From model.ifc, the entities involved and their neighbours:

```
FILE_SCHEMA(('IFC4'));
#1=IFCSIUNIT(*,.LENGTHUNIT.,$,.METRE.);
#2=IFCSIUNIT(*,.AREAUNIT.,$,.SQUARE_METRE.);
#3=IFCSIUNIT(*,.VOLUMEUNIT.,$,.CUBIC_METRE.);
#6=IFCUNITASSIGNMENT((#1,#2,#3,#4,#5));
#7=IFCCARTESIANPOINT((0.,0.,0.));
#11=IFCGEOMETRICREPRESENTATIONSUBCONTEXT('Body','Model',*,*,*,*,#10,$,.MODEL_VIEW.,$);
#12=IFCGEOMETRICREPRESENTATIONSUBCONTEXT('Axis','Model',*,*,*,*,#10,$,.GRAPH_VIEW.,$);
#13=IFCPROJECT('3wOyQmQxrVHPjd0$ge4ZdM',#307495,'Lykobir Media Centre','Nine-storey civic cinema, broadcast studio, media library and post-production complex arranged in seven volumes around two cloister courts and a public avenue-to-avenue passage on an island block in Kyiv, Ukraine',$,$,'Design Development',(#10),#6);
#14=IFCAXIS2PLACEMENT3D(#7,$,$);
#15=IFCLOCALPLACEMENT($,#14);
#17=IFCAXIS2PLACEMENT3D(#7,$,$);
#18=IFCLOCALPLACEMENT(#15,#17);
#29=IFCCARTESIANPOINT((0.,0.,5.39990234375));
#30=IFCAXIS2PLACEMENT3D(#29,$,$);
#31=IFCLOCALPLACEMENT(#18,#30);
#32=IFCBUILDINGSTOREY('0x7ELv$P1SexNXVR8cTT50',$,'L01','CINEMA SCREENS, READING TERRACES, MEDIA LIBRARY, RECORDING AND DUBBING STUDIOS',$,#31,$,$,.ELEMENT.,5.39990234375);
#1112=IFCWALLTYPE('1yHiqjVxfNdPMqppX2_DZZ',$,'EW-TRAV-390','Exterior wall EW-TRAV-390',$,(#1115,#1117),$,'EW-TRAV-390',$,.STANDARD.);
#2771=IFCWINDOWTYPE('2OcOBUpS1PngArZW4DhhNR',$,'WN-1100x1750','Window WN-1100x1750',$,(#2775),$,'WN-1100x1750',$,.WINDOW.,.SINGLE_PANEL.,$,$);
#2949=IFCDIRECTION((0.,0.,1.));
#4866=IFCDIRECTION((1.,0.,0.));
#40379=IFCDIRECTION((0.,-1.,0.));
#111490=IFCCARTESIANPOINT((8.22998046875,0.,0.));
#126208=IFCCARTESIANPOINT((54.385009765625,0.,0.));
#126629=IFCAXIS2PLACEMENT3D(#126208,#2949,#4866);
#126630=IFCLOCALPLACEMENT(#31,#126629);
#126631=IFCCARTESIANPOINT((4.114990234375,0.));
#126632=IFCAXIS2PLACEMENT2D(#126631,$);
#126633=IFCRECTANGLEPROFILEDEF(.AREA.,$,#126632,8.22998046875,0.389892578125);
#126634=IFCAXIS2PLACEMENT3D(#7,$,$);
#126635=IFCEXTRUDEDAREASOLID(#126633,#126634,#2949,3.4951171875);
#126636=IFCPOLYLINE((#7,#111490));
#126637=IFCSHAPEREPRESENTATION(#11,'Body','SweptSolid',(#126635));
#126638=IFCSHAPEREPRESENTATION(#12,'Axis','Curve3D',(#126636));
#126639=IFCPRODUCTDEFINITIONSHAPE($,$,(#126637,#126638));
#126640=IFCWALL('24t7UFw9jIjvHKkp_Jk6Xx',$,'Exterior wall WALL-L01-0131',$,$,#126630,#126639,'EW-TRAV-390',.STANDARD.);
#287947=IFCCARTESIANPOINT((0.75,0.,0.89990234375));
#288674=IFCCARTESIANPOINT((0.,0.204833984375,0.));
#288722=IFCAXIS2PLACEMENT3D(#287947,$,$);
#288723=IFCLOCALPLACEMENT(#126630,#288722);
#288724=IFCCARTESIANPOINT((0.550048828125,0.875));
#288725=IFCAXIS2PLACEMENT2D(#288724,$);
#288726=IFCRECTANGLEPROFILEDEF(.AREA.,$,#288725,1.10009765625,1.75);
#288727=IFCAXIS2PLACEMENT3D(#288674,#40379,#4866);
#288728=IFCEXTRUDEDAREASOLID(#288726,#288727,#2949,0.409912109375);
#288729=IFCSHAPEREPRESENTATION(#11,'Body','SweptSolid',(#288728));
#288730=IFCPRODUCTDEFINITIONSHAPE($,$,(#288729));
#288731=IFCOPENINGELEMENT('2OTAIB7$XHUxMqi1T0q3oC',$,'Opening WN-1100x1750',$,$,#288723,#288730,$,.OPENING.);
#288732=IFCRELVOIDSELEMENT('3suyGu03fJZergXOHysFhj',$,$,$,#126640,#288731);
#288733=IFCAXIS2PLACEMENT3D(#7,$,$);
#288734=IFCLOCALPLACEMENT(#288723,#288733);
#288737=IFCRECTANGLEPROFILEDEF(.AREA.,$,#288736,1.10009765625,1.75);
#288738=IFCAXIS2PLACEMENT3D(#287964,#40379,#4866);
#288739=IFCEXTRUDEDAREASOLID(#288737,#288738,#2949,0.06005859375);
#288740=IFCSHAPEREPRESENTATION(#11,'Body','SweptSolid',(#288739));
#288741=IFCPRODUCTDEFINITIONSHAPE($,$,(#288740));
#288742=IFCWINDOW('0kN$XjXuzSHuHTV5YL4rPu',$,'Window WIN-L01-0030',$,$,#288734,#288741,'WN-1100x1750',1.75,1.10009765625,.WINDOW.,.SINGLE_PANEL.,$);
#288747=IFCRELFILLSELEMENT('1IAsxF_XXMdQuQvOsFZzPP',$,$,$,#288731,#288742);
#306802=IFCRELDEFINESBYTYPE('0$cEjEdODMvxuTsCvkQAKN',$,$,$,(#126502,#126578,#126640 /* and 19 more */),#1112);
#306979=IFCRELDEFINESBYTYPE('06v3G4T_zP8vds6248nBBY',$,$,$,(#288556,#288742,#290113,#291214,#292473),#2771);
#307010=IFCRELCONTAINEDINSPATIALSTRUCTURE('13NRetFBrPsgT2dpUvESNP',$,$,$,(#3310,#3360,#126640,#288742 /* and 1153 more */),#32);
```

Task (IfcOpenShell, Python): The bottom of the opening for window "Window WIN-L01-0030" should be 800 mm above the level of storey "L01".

```python
import numpy as np
import ifcopenshell
import ifcopenshell.api.geometry
import ifcopenshell.geom
import ifcopenshell.util.element
import ifcopenshell.util.placement
import ifcopenshell.util.shape
import ifcopenshell.util.unit

model = ifcopenshell.open("model.ifc")
unit_scale = ifcopenshell.util.unit.calculate_unit_scale(model)

window = model.by_guid("0kN$XjXuzSHuHTV5YL4rPu")
opening = window.FillsVoids[0].RelatingOpeningElement
storey = ifcopenshell.util.element.get_container(window, ifc_class="IfcBuildingStorey")
level = ifcopenshell.util.placement.get_local_placement(storey.ObjectPlacement)[2, 3]

# The opening's origin need not be at the sill, so measure its lowest point.
shape = ifcopenshell.geom.create_shape(ifcopenshell.geom.settings(), opening)
bottom = ifcopenshell.util.shape.get_shape_bottom_elevation(shape, shape.geometry) / unit_scale
dz = level + 0.8 - bottom

shift = np.array([0.0, 0.0, dz])
# The window is placed relative to its opening, so it follows when the opening moves.
matrix = ifcopenshell.util.placement.get_local_placement(opening.ObjectPlacement)
matrix[:3, 3] += shift
ifcopenshell.api.geometry.edit_object_placement(
    model, product=opening, matrix=matrix, is_si=False, should_transform_children=True
)

print(f"moved by {dz * unit_scale:+.3f} m")

model.write("model_updated.ifc")
```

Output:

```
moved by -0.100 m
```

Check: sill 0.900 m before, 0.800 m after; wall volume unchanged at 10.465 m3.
